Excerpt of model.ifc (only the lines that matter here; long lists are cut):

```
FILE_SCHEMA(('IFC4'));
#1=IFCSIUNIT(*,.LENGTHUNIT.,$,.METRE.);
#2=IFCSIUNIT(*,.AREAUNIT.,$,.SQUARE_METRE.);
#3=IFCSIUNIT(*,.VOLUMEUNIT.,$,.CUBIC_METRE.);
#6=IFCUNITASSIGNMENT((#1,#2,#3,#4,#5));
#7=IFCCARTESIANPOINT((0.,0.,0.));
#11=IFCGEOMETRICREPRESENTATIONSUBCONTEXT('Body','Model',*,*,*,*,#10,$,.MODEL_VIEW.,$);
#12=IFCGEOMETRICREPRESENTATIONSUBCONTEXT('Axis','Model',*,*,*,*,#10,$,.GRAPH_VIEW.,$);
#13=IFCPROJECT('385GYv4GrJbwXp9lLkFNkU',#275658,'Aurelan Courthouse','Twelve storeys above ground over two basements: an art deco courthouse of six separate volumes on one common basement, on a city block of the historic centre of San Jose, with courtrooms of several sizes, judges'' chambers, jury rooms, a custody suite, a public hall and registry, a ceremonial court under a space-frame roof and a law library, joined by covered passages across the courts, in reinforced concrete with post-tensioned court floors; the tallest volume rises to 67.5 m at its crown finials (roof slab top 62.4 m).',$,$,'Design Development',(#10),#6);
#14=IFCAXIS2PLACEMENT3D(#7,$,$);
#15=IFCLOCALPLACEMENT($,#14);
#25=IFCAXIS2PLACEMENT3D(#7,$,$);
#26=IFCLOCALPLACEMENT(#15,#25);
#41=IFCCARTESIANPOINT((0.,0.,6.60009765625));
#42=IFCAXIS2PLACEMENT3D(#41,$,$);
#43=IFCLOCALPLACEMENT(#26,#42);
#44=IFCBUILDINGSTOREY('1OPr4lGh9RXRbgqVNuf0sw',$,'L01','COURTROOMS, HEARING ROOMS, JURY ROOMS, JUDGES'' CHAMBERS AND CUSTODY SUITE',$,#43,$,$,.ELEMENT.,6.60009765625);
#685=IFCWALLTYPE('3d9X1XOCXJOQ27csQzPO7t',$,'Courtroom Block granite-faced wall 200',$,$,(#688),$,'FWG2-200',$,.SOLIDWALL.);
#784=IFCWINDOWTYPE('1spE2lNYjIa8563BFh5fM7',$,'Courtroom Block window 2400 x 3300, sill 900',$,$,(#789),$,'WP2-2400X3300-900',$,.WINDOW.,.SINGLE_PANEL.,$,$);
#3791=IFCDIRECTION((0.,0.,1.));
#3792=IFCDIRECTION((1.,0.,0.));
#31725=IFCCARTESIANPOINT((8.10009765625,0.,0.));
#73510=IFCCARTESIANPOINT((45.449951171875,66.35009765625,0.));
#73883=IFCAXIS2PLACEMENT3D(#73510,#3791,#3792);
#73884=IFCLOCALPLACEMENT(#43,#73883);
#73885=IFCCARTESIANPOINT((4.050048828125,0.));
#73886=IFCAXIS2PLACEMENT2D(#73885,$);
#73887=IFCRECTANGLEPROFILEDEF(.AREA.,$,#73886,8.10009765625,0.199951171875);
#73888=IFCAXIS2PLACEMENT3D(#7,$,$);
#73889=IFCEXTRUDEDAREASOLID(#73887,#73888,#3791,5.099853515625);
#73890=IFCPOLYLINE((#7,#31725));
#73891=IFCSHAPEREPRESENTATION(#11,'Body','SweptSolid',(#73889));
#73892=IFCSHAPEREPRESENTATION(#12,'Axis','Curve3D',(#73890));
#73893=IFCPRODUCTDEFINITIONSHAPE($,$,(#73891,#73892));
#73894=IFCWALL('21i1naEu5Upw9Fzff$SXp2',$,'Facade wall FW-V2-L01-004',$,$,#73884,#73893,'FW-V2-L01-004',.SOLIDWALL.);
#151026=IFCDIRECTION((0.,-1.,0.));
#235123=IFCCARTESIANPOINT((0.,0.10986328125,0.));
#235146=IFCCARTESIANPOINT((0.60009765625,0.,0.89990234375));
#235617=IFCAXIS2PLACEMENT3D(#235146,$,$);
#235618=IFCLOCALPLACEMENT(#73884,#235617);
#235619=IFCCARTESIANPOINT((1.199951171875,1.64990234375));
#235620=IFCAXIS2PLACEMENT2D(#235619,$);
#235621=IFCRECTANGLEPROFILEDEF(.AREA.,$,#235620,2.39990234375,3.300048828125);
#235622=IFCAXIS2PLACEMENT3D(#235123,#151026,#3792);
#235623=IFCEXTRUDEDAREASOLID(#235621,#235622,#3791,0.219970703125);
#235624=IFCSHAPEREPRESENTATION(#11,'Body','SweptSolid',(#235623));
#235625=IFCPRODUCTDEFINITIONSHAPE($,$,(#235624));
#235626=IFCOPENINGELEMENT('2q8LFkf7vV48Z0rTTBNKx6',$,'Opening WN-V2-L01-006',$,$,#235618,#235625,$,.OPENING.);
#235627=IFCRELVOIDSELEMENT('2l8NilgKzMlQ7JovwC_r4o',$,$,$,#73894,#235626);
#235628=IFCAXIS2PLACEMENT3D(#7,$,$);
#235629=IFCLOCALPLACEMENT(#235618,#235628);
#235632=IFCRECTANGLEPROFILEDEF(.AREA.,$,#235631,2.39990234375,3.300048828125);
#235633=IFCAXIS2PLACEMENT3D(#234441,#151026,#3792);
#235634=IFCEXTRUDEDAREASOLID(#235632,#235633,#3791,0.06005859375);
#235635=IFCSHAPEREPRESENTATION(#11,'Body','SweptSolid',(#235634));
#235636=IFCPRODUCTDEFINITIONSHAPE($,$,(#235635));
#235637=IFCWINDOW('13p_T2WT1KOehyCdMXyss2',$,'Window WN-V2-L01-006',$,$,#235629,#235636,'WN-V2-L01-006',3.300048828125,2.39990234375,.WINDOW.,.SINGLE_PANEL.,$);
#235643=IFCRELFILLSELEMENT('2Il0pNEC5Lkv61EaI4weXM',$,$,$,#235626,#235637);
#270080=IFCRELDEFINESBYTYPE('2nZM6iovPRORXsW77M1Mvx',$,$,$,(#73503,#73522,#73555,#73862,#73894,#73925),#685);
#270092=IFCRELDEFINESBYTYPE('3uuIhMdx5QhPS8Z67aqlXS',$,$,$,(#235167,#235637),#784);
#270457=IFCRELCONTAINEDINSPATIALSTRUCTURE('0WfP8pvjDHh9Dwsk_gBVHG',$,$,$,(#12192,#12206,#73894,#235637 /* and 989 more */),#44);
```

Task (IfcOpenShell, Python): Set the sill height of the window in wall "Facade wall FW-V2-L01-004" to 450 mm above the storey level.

```python
import numpy as np
import ifcopenshell
import ifcopenshell.api.geometry
import ifcopenshell.geom
import ifcopenshell.util.element
import ifcopenshell.util.placement
import ifcopenshell.util.shape
import ifcopenshell.util.unit

model = ifcopenshell.open("model.ifc")
unit_scale = ifcopenshell.util.unit.calculate_unit_scale(model)

window = model.by_id(235637)
opening = window.FillsVoids[0].RelatingOpeningElement
storey = ifcopenshell.util.element.get_container(window, ifc_class="IfcBuildingStorey")
level = ifcopenshell.util.placement.get_local_placement(storey.ObjectPlacement)[2, 3]

# The opening's origin need not be at the sill, so measure its lowest point.
shape = ifcopenshell.geom.create_shape(ifcopenshell.geom.settings(), opening)
bottom = ifcopenshell.util.shape.get_shape_bottom_elevation(shape, shape.geometry) / unit_scale
dz = level + 0.45 / unit_scale - bottom

shift = np.array([0.0, 0.0, dz])
# The window is placed relative to its opening, so it follows when the opening moves.
matrix = ifcopenshell.util.placement.get_local_placement(opening.ObjectPlacement)
matrix[:3, 3] += shift
ifcopenshell.api.geometry.edit_object_placement(
    model, product=opening, matrix=matrix, is_si=False, should_transform_children=True
)

print(f"moved by {dz * unit_scale:+.3f} m")

model.write("model-out.ifc")
```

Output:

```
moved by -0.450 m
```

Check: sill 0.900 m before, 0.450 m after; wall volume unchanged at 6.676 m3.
